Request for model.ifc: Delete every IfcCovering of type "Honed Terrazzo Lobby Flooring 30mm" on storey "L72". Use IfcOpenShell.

First a look at what the model holds.

```python
import ifcopenshell
import ifcopenshell.util.element

model = ifcopenshell.open("model.ifc")
print(model.schema)
storey = next(s for s in model.by_type("IfcBuildingStorey") if s.Name == "L72")
coverings = [e for e in ifcopenshell.util.element.get_decomposition(storey) if e.is_a("IfcCovering")]
seen = {}
for e in coverings:
    element_type = ifcopenshell.util.element.get_type(e)
    name = element_type.Name if element_type not in (None, e) else None
    seen[name] = seen.get(name, 0) + 1
for name, count in sorted(seen.items(), key=str):
    print(count, "x", name)
```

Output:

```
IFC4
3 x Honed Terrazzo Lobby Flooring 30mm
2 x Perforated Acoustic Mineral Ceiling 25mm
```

```python
import ifcopenshell
import ifcopenshell.api.root
import ifcopenshell.util.element

model = ifcopenshell.open("model.ifc")

storey = next(s for s in model.by_type("IfcBuildingStorey") if s.Name == "L72")
coverings = [e for e in ifcopenshell.util.element.get_decomposition(storey) if e.is_a("IfcCovering")]
targets = [e for e in coverings if (t := ifcopenshell.util.element.get_type(e)) not in (None, e) and t.Name == "Honed Terrazzo Lobby Flooring 30mm"]

for e in targets:
    ifcopenshell.api.root.remove_product(model, product=e)
print(len(targets), "removed")

model.write("model_updated.ifc")
```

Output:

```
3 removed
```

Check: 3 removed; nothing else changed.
